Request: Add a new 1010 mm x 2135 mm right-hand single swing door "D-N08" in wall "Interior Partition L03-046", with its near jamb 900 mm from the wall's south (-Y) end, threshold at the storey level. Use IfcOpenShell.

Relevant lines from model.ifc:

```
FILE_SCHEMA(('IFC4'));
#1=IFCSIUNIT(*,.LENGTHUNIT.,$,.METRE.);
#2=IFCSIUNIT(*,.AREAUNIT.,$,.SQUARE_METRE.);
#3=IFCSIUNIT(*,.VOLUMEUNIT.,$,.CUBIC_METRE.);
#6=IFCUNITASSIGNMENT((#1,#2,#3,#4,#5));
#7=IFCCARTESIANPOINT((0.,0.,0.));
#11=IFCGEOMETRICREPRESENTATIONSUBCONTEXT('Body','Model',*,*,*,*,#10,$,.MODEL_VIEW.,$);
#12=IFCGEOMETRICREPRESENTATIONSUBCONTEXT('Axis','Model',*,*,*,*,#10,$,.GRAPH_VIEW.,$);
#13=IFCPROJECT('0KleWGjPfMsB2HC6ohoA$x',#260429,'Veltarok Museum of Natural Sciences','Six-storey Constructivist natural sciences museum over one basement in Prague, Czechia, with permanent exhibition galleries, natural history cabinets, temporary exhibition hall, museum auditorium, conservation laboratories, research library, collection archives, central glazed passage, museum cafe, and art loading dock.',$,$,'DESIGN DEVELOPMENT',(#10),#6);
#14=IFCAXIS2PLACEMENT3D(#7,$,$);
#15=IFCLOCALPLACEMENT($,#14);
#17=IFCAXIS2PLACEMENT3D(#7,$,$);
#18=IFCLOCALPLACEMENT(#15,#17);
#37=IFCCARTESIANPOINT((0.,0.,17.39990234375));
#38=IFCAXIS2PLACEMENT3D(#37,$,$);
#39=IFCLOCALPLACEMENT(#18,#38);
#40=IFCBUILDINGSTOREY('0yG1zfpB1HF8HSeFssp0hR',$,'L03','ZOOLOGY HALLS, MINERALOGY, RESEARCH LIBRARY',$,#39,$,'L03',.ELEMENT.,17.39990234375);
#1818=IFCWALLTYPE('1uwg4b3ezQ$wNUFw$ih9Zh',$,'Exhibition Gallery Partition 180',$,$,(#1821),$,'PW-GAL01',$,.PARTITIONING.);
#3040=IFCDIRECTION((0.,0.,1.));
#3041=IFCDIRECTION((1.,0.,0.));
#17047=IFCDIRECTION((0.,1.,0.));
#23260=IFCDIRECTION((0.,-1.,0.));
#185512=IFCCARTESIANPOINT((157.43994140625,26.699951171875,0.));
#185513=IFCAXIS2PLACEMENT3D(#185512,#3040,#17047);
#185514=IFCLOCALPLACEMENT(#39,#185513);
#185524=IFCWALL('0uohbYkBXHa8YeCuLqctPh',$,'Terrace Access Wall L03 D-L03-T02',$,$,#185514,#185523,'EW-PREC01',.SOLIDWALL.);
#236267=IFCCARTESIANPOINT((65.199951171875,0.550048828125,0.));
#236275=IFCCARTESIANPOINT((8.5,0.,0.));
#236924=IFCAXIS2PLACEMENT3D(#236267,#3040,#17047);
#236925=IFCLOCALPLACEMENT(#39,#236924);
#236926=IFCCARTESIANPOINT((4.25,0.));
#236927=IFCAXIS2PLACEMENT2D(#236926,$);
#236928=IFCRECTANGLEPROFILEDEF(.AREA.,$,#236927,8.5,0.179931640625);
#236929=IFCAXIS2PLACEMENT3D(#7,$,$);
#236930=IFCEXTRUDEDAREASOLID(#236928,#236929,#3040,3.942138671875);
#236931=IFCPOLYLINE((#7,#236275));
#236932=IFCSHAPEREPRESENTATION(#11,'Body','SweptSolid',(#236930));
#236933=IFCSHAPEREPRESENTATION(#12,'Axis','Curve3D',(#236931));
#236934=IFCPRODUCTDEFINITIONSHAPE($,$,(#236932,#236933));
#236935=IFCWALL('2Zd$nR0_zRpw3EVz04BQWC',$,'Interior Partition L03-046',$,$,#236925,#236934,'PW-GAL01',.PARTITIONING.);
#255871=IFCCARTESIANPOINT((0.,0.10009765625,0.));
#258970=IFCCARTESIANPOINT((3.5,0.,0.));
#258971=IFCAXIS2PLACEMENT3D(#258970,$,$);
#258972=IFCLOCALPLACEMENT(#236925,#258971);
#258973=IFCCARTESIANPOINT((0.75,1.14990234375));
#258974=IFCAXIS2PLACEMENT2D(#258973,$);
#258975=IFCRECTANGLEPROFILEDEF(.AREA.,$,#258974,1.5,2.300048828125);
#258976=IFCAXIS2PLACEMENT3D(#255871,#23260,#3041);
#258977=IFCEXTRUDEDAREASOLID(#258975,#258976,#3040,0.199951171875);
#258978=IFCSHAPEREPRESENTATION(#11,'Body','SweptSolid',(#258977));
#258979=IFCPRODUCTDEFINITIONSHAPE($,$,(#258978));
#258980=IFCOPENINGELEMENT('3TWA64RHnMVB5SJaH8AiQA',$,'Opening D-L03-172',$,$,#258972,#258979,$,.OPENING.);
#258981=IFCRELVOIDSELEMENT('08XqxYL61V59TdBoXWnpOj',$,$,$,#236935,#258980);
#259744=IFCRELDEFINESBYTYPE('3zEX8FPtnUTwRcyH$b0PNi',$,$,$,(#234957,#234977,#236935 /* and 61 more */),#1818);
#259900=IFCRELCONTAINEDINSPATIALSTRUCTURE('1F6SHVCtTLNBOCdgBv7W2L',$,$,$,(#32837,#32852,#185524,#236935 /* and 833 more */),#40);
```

```python
import numpy as np
import ifcopenshell
import ifcopenshell.api.feature
import ifcopenshell.api.geometry
import ifcopenshell.api.root
import ifcopenshell.api.spatial
import ifcopenshell.geom
import ifcopenshell.util.element
import ifcopenshell.util.placement
import ifcopenshell.util.representation
import ifcopenshell.util.shape
import ifcopenshell.util.unit

model = ifcopenshell.open("model.ifc")
unit_scale = ifcopenshell.util.unit.calculate_unit_scale(model)
settings = ifcopenshell.geom.settings()


def volume(element):
    """Net volume in cubic metres, openings subtracted."""
    shape = ifcopenshell.geom.create_shape(settings, element)
    return ifcopenshell.util.shape.get_volume(shape.geometry)


wall = model.by_guid("2Zd$nR0_zRpw3EVz04BQWC")
storey = ifcopenshell.util.element.get_container(wall, ifc_class="IfcBuildingStorey")
context = ifcopenshell.util.representation.get_context(model, "Model", "Body", "MODEL_VIEW")
before = volume(wall)

width, height, from_end, sill = 1.01, 2.135, 0.9, 0.0  # metres

# The wall runs along its own X axis, and the end named is its -X end.
wall_shape = ifcopenshell.geom.create_shape(settings, wall)
x, y, z = ifcopenshell.util.shape.get_vertices(wall_shape.geometry).T
start = x.min() + from_end
face, thickness = float(y.min()), float(y.max() - y.min())
wall_matrix = ifcopenshell.util.placement.get_local_placement(wall.ObjectPlacement)
level = ifcopenshell.util.placement.get_local_placement(storey.ObjectPlacement)[2, 3]


def in_wall(x, y):
    """Placement at x, y metres in the wall's axes, at sill height."""
    matrix = wall_matrix.copy()
    matrix[:, 3] = wall_matrix @ np.array([x / unit_scale, y / unit_scale, 0.0, 1.0])
    matrix[2, 3] = level + sill / unit_scale
    return matrix


# Opening: a box that overshoots both wall faces by 50 mm.
opening = ifcopenshell.api.root.create_entity(model, ifc_class="IfcOpeningElement", predefined_type="OPENING")
box = ifcopenshell.api.geometry.add_wall_representation(
    model, context=context, length=width, height=height, thickness=thickness + 0.1
)
ifcopenshell.api.geometry.assign_representation(model, product=opening, representation=box)
ifcopenshell.api.geometry.edit_object_placement(model, product=opening, matrix=in_wall(start, face - 0.05), is_si=False)
ifcopenshell.api.feature.add_feature(model, feature=opening, element=wall)

door = ifcopenshell.api.root.create_entity(model, ifc_class="IfcDoor", name="D-N08", predefined_type="DOOR")
door.OverallWidth, door.OverallHeight = width / unit_scale, height / unit_scale
door.OperationType = "SINGLE_SWING_RIGHT"
body = ifcopenshell.api.geometry.add_door_representation(
    model,
    context=context,
    overall_width=door.OverallWidth,
    overall_height=door.OverallHeight,
    operation_type="SINGLE_SWING_RIGHT",
    lining_properties={"LiningDepth": thickness / unit_scale, "ThresholdDepth": thickness / unit_scale},
)
ifcopenshell.api.geometry.assign_representation(model, product=door, representation=body)
ifcopenshell.api.spatial.assign_container(model, products=[door], relating_structure=storey)
ifcopenshell.api.feature.add_filling(model, opening=opening, element=door)

# The lining spans the wall, so the door starts at the wall face.
ifcopenshell.api.geometry.edit_object_placement(model, product=door, matrix=in_wall(start, face), is_si=False)

after = volume(wall)

print(f"wall volume {before:.3f} -> {after:.3f} m3")

model.write("model_rev.ifc")
```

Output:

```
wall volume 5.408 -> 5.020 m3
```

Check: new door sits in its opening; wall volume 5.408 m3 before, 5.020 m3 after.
